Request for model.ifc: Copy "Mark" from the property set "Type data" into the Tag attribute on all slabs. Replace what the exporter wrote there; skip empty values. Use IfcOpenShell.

First a look at what the model holds.

```python
import ifcopenshell
import ifcopenshell.util.element

model = ifcopenshell.open("model.ifc")
print(model.schema)
slabs = model.by_type("IfcSlab")
print(len(slabs), "slabs")
for e in slabs[:8]:
    source = ifcopenshell.util.element.get_pset(e, "Type data", "Mark")
    target = e.Tag
    print(e.id(), repr(source), repr(target), sep=" | ")
```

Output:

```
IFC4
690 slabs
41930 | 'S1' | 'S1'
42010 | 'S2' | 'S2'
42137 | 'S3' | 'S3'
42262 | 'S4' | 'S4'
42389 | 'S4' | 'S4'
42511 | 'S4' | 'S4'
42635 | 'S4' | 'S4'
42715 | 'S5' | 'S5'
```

```python
import ifcopenshell
import ifcopenshell.util.element

model = ifcopenshell.open("model.ifc")

count = 0
for e in model.by_type("IfcSlab"):
    value = ifcopenshell.util.element.get_pset(e, "Type data", "Mark")
    current = e.Tag
    if not value or not value.strip() or current == value:
        continue
    e.Tag = value
    count += 1

print(count, "slabs updated")

model.write("model_rev.ifc")
```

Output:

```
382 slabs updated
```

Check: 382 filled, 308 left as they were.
